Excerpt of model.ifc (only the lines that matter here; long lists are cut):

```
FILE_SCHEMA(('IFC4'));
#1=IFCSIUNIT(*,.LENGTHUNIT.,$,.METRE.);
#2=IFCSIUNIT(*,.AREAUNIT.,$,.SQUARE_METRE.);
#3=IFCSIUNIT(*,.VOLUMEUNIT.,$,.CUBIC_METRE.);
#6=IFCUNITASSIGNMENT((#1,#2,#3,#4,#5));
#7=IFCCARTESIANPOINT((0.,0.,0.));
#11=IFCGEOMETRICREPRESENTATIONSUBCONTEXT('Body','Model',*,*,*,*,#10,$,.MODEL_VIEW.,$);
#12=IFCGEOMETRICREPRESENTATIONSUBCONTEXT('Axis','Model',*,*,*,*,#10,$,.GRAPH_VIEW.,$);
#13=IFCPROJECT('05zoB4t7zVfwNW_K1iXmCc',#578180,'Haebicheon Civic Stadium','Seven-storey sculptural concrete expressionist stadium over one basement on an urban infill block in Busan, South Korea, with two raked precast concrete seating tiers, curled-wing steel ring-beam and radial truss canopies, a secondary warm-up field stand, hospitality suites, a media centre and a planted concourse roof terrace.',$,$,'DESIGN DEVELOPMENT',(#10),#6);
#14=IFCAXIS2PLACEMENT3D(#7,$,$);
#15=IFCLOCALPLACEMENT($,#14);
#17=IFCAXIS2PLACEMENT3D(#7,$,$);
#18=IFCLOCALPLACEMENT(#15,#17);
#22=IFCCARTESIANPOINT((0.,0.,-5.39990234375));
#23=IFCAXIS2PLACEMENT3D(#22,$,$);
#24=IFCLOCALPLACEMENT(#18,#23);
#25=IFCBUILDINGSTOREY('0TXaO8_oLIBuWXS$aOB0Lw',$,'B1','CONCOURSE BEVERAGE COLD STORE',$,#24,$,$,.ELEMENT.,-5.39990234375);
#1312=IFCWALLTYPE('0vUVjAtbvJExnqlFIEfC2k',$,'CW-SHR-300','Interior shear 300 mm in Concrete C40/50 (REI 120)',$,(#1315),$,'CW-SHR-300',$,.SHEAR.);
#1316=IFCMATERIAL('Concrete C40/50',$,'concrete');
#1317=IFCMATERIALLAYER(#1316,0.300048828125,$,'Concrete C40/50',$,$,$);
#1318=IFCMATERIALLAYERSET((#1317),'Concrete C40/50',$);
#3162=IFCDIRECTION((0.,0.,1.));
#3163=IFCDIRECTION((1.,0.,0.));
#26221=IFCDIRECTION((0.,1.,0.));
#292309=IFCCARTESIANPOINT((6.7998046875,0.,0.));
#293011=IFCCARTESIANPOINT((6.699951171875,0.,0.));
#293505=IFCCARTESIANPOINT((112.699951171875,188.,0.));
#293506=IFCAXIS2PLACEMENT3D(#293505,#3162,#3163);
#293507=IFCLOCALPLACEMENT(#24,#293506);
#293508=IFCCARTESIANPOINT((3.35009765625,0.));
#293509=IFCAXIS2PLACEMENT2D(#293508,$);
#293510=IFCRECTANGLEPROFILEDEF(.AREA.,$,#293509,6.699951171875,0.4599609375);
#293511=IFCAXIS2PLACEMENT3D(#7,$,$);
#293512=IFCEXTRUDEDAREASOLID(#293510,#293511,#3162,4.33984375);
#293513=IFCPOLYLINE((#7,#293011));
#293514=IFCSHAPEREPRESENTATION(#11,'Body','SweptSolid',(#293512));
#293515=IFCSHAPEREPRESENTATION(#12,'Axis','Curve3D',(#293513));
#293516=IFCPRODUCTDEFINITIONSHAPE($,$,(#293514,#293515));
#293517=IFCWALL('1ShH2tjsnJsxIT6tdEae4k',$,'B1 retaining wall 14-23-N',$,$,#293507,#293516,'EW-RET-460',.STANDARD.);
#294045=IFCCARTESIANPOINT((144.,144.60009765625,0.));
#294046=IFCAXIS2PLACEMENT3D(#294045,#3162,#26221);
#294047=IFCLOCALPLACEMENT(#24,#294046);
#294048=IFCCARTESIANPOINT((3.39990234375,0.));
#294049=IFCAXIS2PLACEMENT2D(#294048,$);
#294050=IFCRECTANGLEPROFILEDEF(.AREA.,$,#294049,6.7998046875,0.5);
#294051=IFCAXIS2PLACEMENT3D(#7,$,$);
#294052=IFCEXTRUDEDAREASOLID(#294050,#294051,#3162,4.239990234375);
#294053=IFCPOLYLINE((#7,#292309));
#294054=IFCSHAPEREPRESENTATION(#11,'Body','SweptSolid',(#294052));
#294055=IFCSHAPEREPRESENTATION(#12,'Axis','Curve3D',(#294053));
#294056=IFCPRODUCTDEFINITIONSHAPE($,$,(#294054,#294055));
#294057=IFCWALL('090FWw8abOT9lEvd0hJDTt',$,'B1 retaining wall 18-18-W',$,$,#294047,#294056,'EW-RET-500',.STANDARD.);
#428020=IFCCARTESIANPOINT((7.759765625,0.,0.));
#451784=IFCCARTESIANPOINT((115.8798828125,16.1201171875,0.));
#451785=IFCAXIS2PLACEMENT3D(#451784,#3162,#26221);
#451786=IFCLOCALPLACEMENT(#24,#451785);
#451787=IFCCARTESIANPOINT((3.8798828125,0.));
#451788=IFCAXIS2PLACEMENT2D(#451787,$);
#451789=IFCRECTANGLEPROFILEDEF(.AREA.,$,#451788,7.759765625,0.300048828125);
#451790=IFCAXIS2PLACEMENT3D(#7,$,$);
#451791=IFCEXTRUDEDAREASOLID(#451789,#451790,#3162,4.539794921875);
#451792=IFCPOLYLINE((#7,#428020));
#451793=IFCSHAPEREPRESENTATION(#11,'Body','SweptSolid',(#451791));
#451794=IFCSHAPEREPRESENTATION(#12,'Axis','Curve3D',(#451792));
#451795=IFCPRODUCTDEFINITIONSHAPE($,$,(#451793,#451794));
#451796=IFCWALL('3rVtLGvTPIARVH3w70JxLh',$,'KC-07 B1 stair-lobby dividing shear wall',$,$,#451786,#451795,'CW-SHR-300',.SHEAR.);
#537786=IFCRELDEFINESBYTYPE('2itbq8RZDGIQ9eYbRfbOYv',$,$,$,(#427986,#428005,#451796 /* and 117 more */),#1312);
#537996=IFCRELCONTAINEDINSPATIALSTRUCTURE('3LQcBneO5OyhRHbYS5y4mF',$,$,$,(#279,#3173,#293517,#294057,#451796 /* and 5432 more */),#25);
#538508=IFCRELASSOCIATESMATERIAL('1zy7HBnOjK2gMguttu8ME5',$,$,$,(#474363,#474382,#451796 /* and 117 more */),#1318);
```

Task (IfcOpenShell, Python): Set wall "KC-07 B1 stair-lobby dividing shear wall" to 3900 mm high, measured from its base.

```python
import ifcopenshell
import ifcopenshell.geom
import ifcopenshell.util.representation
import ifcopenshell.util.shape
import ifcopenshell.util.unit

model = ifcopenshell.open("model.ifc")
unit_scale = ifcopenshell.util.unit.calculate_unit_scale(model)
settings = ifcopenshell.geom.settings()


def volume(element):
    """Net volume in cubic metres, openings subtracted."""
    shape = ifcopenshell.geom.create_shape(settings, element)
    return ifcopenshell.util.shape.get_volume(shape.geometry)


wall = model.by_id(451796)
before = volume(wall)

body = ifcopenshell.util.representation.get_representation(wall, "Model", "Body")
solid = body.Items[0]
old_height = solid.Depth
solid.Depth = 3.9 / unit_scale
after = volume(wall)

print(f"height {old_height:g} -> {solid.Depth:g}, volume {before:.3f} -> {after:.3f} m3")

model.write("model_edited.ifc")
```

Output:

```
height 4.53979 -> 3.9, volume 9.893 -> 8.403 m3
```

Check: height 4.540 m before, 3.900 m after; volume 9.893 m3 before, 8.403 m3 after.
